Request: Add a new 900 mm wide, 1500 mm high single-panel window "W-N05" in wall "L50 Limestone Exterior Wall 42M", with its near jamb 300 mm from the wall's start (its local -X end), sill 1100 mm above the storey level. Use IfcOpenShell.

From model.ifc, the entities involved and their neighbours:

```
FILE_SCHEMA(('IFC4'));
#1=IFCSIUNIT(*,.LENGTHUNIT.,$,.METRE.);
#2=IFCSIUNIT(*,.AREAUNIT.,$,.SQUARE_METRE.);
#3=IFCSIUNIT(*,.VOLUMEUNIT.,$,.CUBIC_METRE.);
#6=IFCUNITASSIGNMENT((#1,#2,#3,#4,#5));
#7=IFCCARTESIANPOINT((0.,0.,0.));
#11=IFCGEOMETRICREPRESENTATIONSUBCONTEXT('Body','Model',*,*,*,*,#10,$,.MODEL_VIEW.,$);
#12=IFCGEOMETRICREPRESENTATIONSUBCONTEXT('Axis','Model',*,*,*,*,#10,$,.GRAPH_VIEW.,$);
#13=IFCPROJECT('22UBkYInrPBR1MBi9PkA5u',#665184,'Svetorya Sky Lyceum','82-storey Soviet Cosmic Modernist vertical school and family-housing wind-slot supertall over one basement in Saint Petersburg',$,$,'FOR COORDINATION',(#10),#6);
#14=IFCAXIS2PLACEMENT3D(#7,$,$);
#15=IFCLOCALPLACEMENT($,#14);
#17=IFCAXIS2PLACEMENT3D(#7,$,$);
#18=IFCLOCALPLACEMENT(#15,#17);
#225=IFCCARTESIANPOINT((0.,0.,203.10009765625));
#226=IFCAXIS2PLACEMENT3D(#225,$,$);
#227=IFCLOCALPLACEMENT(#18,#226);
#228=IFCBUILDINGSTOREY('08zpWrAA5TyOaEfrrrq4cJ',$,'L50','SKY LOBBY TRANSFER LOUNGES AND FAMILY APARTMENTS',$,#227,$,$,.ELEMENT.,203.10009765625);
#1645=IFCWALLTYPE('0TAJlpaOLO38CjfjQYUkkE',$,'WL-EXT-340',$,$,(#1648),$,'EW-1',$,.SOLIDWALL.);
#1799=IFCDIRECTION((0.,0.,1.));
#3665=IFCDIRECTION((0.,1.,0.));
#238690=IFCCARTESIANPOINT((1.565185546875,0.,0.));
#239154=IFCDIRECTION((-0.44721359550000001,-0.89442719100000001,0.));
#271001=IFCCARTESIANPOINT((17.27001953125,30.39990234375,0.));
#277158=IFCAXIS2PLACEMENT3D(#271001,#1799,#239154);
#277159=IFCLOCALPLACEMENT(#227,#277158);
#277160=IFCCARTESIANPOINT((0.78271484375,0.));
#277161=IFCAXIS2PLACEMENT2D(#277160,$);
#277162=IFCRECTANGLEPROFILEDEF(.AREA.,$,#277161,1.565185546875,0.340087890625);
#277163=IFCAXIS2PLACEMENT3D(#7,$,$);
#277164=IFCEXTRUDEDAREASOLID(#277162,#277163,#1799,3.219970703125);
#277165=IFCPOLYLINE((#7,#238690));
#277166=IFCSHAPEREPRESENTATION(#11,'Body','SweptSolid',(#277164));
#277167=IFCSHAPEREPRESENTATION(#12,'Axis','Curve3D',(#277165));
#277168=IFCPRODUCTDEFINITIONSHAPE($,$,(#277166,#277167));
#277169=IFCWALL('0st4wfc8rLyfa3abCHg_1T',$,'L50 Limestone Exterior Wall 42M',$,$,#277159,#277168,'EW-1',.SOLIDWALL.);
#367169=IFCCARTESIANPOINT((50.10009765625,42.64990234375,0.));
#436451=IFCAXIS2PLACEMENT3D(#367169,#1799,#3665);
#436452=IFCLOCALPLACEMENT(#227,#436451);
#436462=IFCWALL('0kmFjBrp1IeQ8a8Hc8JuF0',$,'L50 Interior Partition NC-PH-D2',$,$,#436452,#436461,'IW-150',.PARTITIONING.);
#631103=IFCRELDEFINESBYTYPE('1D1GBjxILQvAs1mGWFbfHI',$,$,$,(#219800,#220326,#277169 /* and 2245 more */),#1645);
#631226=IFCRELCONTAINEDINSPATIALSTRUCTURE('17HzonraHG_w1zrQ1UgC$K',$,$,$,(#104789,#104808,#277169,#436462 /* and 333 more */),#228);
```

```python
import numpy as np
import ifcopenshell
import ifcopenshell.api.feature
import ifcopenshell.api.geometry
import ifcopenshell.api.root
import ifcopenshell.api.spatial
import ifcopenshell.geom
import ifcopenshell.util.element
import ifcopenshell.util.placement
import ifcopenshell.util.representation
import ifcopenshell.util.shape
import ifcopenshell.util.unit

model = ifcopenshell.open("model.ifc")
unit_scale = ifcopenshell.util.unit.calculate_unit_scale(model)
settings = ifcopenshell.geom.settings()


def volume(element):
    """Net volume in cubic metres, openings subtracted."""
    shape = ifcopenshell.geom.create_shape(settings, element)
    return ifcopenshell.util.shape.get_volume(shape.geometry)


wall = model.by_id(277169)
storey = ifcopenshell.util.element.get_container(wall, ifc_class="IfcBuildingStorey")
context = ifcopenshell.util.representation.get_context(model, "Model", "Body", "MODEL_VIEW")
before = volume(wall)

width, height, from_end, sill = 0.9, 1.5, 0.3, 1.1  # metres

# The wall runs along its own X axis, and the end named is its -X end.
wall_shape = ifcopenshell.geom.create_shape(settings, wall)
x, y, z = ifcopenshell.util.shape.get_vertices(wall_shape.geometry).T
start = x.min() + from_end
face, thickness = float(y.min()), float(y.max() - y.min())
wall_matrix = ifcopenshell.util.placement.get_local_placement(wall.ObjectPlacement)
level = ifcopenshell.util.placement.get_local_placement(storey.ObjectPlacement)[2, 3]


def in_wall(x, y):
    """Placement at x, y metres in the wall's axes, at sill height."""
    matrix = wall_matrix.copy()
    matrix[:, 3] = wall_matrix @ np.array([x / unit_scale, y / unit_scale, 0.0, 1.0])
    matrix[2, 3] = level + sill / unit_scale
    return matrix


# Opening: a box that overshoots both wall faces by 50 mm.
opening = ifcopenshell.api.root.create_entity(model, ifc_class="IfcOpeningElement", predefined_type="OPENING")
box = ifcopenshell.api.geometry.add_wall_representation(
    model, context=context, length=width, height=height, thickness=thickness + 0.1
)
ifcopenshell.api.geometry.assign_representation(model, product=opening, representation=box)
ifcopenshell.api.geometry.edit_object_placement(model, product=opening, matrix=in_wall(start, face - 0.05), is_si=False)
ifcopenshell.api.feature.add_feature(model, feature=opening, element=wall)

window = ifcopenshell.api.root.create_entity(model, ifc_class="IfcWindow", name="W-N05", predefined_type="WINDOW")
window.OverallWidth, window.OverallHeight = width / unit_scale, height / unit_scale
window.PartitioningType = "SINGLE_PANEL"
body = ifcopenshell.api.geometry.add_window_representation(
    model,
    context=context,
    overall_width=window.OverallWidth,
    overall_height=window.OverallHeight,
    partition_type="SINGLE_PANEL",
)
ifcopenshell.api.geometry.assign_representation(model, product=window, representation=body)
ifcopenshell.api.spatial.assign_container(model, products=[window], relating_structure=storey)
ifcopenshell.api.feature.add_filling(model, opening=opening, element=window)

# Centre the window in the wall's thickness.
ifcopenshell.api.geometry.edit_object_placement(model, product=window, matrix=in_wall(start, face), is_si=False)
window_shape = ifcopenshell.geom.create_shape(settings, window)
depth = ifcopenshell.util.shape.get_vertices(window_shape.geometry)[:, 1]
offset = face + thickness / 2 - (depth.min() + depth.max()) / 2
ifcopenshell.api.geometry.edit_object_placement(model, product=window, matrix=in_wall(start, offset), is_si=False)

after = volume(wall)

print(f"wall volume {before:.3f} -> {after:.3f} m3")

model.write("model-out.ifc")
```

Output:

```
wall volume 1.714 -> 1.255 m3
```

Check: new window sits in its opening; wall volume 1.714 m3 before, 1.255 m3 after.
